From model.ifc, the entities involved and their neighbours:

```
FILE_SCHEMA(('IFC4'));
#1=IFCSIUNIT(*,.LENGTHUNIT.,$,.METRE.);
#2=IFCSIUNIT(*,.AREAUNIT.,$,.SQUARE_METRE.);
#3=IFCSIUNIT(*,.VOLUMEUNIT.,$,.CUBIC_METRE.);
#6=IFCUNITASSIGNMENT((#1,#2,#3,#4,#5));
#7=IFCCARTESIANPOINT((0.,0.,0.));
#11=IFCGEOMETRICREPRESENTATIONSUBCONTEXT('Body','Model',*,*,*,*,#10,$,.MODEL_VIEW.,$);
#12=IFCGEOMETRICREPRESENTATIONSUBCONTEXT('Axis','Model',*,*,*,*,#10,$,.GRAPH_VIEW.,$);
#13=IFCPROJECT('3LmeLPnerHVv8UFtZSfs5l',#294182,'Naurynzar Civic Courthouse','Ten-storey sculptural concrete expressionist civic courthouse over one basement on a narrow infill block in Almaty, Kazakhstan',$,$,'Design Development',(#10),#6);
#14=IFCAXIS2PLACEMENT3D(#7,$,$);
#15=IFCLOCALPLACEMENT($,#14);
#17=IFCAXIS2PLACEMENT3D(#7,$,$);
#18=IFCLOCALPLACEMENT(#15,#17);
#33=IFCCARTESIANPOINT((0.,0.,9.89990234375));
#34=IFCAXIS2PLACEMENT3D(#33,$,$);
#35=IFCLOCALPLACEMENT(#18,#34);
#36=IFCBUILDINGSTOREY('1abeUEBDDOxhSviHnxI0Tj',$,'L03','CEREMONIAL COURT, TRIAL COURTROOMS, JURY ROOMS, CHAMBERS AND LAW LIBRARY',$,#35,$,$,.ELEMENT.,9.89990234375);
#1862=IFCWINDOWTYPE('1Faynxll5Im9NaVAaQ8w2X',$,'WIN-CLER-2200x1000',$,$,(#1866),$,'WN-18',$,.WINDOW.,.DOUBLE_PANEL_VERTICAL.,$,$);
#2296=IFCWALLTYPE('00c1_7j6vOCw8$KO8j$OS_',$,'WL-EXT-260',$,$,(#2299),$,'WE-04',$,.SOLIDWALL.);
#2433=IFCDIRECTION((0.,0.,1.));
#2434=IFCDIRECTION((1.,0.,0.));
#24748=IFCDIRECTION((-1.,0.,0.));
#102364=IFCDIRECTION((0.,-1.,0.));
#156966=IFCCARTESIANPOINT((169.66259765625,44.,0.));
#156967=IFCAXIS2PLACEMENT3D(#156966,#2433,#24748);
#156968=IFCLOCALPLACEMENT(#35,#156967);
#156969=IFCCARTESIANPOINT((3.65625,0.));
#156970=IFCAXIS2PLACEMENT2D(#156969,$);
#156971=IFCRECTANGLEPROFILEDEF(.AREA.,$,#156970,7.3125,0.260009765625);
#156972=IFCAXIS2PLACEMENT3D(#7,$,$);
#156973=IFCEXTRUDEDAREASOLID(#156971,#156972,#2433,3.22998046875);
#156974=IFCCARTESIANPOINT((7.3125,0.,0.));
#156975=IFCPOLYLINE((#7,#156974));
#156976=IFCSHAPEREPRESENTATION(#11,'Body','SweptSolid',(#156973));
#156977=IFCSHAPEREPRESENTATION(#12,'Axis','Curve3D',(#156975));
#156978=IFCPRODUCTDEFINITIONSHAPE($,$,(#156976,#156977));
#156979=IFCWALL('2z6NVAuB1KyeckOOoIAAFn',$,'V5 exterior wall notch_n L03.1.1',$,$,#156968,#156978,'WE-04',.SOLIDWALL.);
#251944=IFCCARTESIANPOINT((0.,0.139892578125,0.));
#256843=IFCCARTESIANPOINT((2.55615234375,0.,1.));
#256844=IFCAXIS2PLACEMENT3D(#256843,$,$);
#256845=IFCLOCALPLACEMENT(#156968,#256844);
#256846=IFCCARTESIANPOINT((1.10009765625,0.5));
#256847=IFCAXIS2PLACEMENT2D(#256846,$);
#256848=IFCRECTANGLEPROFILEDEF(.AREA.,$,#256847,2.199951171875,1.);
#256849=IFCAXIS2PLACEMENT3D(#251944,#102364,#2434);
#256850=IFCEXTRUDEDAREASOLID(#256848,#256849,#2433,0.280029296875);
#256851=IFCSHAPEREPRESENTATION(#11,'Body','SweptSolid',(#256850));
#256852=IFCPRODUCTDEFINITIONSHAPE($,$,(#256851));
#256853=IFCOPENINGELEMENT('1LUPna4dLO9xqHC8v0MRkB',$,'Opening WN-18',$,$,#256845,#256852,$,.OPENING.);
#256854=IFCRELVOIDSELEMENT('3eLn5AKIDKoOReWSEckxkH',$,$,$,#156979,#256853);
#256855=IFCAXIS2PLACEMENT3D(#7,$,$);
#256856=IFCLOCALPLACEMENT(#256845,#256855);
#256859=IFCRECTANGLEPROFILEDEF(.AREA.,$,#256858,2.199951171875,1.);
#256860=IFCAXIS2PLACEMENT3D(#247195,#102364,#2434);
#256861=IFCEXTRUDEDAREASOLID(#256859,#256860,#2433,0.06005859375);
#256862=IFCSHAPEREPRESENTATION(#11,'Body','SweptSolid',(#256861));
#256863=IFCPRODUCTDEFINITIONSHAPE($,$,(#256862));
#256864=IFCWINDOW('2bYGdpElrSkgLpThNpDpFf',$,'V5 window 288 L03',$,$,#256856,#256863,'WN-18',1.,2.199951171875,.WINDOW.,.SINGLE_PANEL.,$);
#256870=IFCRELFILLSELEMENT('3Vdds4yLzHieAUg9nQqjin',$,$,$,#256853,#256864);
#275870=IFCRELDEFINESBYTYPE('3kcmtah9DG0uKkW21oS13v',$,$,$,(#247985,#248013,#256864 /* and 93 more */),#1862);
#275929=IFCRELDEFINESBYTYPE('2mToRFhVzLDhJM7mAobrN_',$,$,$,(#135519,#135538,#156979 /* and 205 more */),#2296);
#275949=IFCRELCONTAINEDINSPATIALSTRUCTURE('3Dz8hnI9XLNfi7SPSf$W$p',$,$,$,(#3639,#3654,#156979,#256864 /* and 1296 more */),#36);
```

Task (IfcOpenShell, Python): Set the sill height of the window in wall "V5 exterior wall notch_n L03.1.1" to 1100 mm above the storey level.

```python
import numpy as np
import ifcopenshell
import ifcopenshell.api.geometry
import ifcopenshell.geom
import ifcopenshell.util.element
import ifcopenshell.util.placement
import ifcopenshell.util.shape
import ifcopenshell.util.unit

model = ifcopenshell.open("model.ifc")
unit_scale = ifcopenshell.util.unit.calculate_unit_scale(model)

window = model.by_guid("2bYGdpElrSkgLpThNpDpFf")
opening = window.FillsVoids[0].RelatingOpeningElement
storey = ifcopenshell.util.element.get_container(window, ifc_class="IfcBuildingStorey")
level = ifcopenshell.util.placement.get_local_placement(storey.ObjectPlacement)[2, 3]

# The opening's origin need not be at the sill, so measure its lowest point.
shape = ifcopenshell.geom.create_shape(ifcopenshell.geom.settings(), opening)
bottom = ifcopenshell.util.shape.get_shape_bottom_elevation(shape, shape.geometry) / unit_scale
dz = level + 1.1 - bottom

shift = np.array([0.0, 0.0, dz])
# The window is placed relative to its opening, so it follows when the opening moves.
matrix = ifcopenshell.util.placement.get_local_placement(opening.ObjectPlacement)
matrix[:3, 3] += shift
ifcopenshell.api.geometry.edit_object_placement(
    model, product=opening, matrix=matrix, is_si=False, should_transform_children=True
)

print(f"moved by {dz * unit_scale:+.3f} m")

model.write("model_edited.ifc")
```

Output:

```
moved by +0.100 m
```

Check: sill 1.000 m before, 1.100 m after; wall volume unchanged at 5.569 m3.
